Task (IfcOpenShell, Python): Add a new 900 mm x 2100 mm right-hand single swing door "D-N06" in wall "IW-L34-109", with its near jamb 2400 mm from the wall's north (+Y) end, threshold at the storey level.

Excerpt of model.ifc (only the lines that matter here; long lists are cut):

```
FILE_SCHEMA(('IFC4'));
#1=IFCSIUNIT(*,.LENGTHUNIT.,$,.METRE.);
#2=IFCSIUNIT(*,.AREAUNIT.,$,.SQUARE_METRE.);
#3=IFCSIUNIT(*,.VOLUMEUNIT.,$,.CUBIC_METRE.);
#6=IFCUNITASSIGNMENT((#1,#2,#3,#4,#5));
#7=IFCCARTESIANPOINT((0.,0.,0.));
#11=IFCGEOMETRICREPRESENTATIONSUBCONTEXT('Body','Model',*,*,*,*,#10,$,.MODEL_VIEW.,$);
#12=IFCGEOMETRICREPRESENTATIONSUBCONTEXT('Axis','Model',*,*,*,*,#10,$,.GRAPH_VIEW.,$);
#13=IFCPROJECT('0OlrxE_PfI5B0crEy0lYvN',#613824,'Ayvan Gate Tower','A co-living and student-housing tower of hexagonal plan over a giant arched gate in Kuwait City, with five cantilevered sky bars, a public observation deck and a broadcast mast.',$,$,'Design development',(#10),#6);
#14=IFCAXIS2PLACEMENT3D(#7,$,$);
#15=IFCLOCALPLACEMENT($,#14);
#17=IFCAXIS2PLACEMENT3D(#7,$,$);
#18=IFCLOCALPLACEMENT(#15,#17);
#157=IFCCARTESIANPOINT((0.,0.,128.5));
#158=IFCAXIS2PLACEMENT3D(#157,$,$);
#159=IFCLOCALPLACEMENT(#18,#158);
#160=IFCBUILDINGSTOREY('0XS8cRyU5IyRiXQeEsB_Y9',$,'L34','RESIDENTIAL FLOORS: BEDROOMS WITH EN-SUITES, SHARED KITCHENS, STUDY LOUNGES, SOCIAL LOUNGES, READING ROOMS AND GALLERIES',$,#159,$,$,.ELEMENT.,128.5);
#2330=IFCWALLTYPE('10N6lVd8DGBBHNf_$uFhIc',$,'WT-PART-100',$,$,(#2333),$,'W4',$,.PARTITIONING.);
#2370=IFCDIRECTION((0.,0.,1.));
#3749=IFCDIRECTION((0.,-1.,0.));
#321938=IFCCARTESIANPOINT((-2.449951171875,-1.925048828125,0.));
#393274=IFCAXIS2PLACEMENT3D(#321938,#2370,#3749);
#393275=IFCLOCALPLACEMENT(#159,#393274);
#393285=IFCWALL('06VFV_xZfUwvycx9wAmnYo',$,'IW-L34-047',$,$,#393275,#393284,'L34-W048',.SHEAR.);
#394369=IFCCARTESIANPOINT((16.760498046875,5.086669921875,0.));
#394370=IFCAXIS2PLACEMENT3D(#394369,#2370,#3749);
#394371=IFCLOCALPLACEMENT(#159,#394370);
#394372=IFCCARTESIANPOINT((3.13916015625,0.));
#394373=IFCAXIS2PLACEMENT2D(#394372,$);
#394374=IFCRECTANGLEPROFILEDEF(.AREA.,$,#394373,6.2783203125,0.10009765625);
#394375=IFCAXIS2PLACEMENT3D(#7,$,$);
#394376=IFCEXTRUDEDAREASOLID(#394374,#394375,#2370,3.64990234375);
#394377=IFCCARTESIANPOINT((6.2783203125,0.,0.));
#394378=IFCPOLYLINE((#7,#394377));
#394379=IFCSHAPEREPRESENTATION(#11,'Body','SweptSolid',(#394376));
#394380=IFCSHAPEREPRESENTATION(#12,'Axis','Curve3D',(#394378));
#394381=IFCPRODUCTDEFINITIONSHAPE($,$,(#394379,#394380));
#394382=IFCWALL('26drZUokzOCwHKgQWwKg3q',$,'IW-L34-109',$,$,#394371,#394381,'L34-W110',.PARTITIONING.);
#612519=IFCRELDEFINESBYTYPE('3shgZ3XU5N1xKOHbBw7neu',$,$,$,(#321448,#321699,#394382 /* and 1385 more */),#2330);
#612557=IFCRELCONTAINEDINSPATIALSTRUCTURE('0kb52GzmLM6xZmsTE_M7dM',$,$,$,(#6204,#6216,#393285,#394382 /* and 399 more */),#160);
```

```python
import numpy as np
import ifcopenshell
import ifcopenshell.api.feature
import ifcopenshell.api.geometry
import ifcopenshell.api.root
import ifcopenshell.api.spatial
import ifcopenshell.geom
import ifcopenshell.util.element
import ifcopenshell.util.placement
import ifcopenshell.util.representation
import ifcopenshell.util.shape
import ifcopenshell.util.unit

model = ifcopenshell.open("model.ifc")
unit_scale = ifcopenshell.util.unit.calculate_unit_scale(model)
settings = ifcopenshell.geom.settings()


def volume(element):
    """Net volume in cubic metres, openings subtracted."""
    shape = ifcopenshell.geom.create_shape(settings, element)
    return ifcopenshell.util.shape.get_volume(shape.geometry)


wall = model.by_id(394382)
storey = ifcopenshell.util.element.get_container(wall, ifc_class="IfcBuildingStorey")
context = ifcopenshell.util.representation.get_context(model, "Model", "Body", "MODEL_VIEW")
before = volume(wall)

width, height, from_end, sill = 0.9, 2.1, 2.4, 0.0  # metres

# The wall runs along its own X axis, and the end named is its -X end.
wall_shape = ifcopenshell.geom.create_shape(settings, wall)
x, y, z = ifcopenshell.util.shape.get_vertices(wall_shape.geometry).T
start = x.min() + from_end
face, thickness = float(y.min()), float(y.max() - y.min())
wall_matrix = ifcopenshell.util.placement.get_local_placement(wall.ObjectPlacement)
level = ifcopenshell.util.placement.get_local_placement(storey.ObjectPlacement)[2, 3]


def in_wall(x, y):
    """Placement at x, y metres in the wall's axes, at sill height."""
    matrix = wall_matrix.copy()
    matrix[:, 3] = wall_matrix @ np.array([x / unit_scale, y / unit_scale, 0.0, 1.0])
    matrix[2, 3] = level + sill / unit_scale
    return matrix


# Opening: a box that overshoots both wall faces by 50 mm.
opening = ifcopenshell.api.root.create_entity(model, ifc_class="IfcOpeningElement", predefined_type="OPENING")
box = ifcopenshell.api.geometry.add_wall_representation(
    model, context=context, length=width, height=height, thickness=thickness + 0.1
)
ifcopenshell.api.geometry.assign_representation(model, product=opening, representation=box)
ifcopenshell.api.geometry.edit_object_placement(model, product=opening, matrix=in_wall(start, face - 0.05), is_si=False)
ifcopenshell.api.feature.add_feature(model, feature=opening, element=wall)

door = ifcopenshell.api.root.create_entity(model, ifc_class="IfcDoor", name="D-N06", predefined_type="DOOR")
door.OverallWidth, door.OverallHeight = width / unit_scale, height / unit_scale
door.OperationType = "SINGLE_SWING_RIGHT"
body = ifcopenshell.api.geometry.add_door_representation(
    model,
    context=context,
    overall_width=door.OverallWidth,
    overall_height=door.OverallHeight,
    operation_type="SINGLE_SWING_RIGHT",
    lining_properties={"LiningDepth": thickness / unit_scale, "ThresholdDepth": thickness / unit_scale},
)
ifcopenshell.api.geometry.assign_representation(model, product=door, representation=body)
ifcopenshell.api.spatial.assign_container(model, products=[door], relating_structure=storey)
ifcopenshell.api.feature.add_filling(model, opening=opening, element=door)

# The lining spans the wall, so the door starts at the wall face.
ifcopenshell.api.geometry.edit_object_placement(model, product=door, matrix=in_wall(start, face), is_si=False)

after = volume(wall)

print(f"wall volume {before:.3f} -> {after:.3f} m3")

model.write("model_rev.ifc")
```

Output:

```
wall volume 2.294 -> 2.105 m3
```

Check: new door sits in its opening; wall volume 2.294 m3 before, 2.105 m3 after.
